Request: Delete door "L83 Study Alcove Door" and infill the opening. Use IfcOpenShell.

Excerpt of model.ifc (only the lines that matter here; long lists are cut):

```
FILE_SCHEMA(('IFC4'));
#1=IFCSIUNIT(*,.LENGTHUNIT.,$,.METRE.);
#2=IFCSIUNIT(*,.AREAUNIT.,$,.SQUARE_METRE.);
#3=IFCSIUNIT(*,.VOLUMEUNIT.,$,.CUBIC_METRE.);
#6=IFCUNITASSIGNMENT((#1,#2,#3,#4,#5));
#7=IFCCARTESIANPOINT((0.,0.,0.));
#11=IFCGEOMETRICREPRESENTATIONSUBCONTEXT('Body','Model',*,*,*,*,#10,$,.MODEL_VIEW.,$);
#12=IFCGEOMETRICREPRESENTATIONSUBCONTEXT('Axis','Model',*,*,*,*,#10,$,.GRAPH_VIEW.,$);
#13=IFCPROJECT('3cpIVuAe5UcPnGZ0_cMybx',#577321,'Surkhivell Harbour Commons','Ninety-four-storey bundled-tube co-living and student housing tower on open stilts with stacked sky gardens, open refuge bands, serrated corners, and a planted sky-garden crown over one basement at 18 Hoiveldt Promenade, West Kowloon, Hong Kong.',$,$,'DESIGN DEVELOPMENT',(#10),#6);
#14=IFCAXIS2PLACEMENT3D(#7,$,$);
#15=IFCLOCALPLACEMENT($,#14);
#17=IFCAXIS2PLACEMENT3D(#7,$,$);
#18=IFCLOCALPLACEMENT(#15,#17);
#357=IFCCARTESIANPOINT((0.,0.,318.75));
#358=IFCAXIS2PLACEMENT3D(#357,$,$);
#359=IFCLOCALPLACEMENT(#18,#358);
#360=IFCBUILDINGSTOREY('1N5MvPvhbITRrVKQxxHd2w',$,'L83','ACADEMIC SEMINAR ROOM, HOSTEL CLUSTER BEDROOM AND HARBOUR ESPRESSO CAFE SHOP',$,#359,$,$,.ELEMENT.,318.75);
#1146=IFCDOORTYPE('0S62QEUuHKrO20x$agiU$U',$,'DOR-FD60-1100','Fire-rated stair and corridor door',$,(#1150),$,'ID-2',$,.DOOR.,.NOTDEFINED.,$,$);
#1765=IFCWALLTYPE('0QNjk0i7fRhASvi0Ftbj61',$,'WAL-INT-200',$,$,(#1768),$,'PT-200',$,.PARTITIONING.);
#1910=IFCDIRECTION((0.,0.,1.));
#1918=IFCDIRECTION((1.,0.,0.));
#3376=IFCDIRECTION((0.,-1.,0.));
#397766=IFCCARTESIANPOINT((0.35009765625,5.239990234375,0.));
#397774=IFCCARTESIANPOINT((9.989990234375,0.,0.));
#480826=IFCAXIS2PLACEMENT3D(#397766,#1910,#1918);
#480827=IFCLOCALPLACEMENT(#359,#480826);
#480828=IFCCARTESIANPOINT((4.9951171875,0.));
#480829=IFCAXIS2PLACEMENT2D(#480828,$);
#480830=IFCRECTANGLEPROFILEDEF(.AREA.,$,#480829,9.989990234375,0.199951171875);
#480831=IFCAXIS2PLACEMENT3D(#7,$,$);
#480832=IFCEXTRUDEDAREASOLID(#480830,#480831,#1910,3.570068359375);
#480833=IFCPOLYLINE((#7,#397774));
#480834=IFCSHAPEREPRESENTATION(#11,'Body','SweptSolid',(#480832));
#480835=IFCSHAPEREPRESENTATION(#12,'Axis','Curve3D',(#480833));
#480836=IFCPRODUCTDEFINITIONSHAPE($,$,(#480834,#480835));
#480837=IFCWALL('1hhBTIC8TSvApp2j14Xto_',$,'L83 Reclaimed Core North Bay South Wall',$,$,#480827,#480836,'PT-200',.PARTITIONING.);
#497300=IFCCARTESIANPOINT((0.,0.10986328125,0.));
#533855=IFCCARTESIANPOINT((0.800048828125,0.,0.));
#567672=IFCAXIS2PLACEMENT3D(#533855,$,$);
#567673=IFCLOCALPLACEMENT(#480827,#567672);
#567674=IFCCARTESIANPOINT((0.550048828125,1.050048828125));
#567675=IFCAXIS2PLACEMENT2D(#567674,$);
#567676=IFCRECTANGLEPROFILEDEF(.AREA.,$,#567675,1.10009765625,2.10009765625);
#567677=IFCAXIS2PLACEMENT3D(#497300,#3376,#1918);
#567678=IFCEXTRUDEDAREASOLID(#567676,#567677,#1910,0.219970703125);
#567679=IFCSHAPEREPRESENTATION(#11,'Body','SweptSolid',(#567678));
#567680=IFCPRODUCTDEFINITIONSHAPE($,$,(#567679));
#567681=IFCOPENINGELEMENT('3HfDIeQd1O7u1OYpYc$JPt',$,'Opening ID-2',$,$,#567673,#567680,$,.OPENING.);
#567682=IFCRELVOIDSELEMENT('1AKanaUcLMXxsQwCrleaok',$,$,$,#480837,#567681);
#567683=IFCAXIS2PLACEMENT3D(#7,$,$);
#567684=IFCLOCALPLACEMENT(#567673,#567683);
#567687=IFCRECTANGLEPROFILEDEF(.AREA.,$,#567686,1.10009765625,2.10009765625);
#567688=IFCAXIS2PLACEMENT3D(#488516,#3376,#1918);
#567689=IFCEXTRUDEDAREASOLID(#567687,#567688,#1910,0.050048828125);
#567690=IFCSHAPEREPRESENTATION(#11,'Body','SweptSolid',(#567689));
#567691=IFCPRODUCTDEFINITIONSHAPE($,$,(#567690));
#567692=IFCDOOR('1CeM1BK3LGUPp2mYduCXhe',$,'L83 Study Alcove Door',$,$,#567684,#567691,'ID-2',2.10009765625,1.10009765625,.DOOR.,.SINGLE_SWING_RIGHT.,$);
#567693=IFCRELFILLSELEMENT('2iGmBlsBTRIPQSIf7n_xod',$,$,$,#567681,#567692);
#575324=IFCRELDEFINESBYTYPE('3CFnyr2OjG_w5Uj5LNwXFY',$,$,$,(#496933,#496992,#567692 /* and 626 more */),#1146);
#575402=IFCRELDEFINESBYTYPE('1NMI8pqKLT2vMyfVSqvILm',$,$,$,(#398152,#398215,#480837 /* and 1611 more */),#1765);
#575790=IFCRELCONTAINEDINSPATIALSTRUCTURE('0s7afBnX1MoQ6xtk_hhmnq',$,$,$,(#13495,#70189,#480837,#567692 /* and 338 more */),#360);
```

```python
import ifcopenshell
import ifcopenshell.api.feature
import ifcopenshell.api.root
import ifcopenshell.geom
import ifcopenshell.util.shape

model = ifcopenshell.open("model.ifc")
settings = ifcopenshell.geom.settings()


def volume(element):
    """Net volume in cubic metres, openings subtracted."""
    shape = ifcopenshell.geom.create_shape(settings, element)
    return ifcopenshell.util.shape.get_volume(shape.geometry)


door = model.by_guid("1CeM1BK3LGUPp2mYduCXhe")
opening = door.FillsVoids[0].RelatingOpeningElement
wall = opening.VoidsElements[0].RelatingBuildingElement
before = volume(wall)

ifcopenshell.api.root.remove_product(model, product=door)
ifcopenshell.api.feature.remove_feature(model, feature=opening)

after = volume(wall)

print(f"wall volume {before:.3f} -> {after:.3f} m3")

model.write("model_edited.ifc")
```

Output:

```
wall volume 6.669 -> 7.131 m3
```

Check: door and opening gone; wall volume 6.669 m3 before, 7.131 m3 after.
